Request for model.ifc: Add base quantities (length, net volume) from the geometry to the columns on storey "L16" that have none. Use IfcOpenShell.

First a look at what the model holds.

```python
import ifcopenshell
import ifcopenshell.util.element
import ifcopenshell.util.unit

model = ifcopenshell.open("model.ifc")
print(model.schema)
for unit_type in ("LENGTHUNIT", "AREAUNIT", "VOLUMEUNIT"):
    print(unit_type, ifcopenshell.util.unit.calculate_unit_scale(model, unit_type))
storey = next(s for s in model.by_type("IfcBuildingStorey") if s.Name == "L16")
columns = [e for e in ifcopenshell.util.element.get_decomposition(storey) if e.is_a("IfcColumn")]
for e in sorted(columns, key=lambda e: e.id()):
    print(e.id(), e.is_a(), e.Name, list(ifcopenshell.util.element.get_psets(e, qtos_only=True)), sep=" | ")
```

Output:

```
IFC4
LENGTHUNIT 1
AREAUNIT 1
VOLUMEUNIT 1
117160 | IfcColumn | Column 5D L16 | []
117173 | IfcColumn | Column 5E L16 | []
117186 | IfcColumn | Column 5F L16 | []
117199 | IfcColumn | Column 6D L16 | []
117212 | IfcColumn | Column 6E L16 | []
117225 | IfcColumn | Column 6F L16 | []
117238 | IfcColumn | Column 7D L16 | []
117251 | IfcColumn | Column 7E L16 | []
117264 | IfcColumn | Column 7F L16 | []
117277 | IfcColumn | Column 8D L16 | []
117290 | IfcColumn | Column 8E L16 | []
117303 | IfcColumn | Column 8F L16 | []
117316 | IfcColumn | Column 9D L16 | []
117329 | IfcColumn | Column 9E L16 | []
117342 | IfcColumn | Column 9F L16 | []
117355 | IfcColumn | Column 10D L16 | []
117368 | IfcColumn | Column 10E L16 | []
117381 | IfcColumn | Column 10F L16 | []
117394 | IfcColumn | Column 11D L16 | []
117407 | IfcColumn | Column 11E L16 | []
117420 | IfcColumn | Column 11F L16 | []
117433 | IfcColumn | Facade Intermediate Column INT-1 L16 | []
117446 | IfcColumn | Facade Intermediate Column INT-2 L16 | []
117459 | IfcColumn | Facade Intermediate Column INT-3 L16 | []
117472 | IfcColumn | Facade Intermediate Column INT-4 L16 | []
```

```python
import ifcopenshell
import ifcopenshell.api.pset
import ifcopenshell.geom
import ifcopenshell.util.element
import ifcopenshell.util.shape
import ifcopenshell.util.unit

model = ifcopenshell.open("model.ifc")
unit_scale = ifcopenshell.util.unit.calculate_unit_scale(model)
volume_scale = ifcopenshell.util.unit.calculate_unit_scale(model, "VOLUMEUNIT")
settings = ifcopenshell.geom.settings()

storey = next(s for s in model.by_type("IfcBuildingStorey") if s.Name == "L16")
columns = [e for e in ifcopenshell.util.element.get_decomposition(storey) if e.is_a("IfcColumn")]

for e in sorted(columns, key=lambda e: e.id()):
    if ifcopenshell.util.element.get_psets(e, qtos_only=True, should_inherit=False):
        continue
    # Geometry comes back in metres, in the element's own axes.
    shape = ifcopenshell.geom.create_shape(settings, e)
    values = {
        "Length": ifcopenshell.util.shape.get_z(shape.geometry) / unit_scale,
        "NetVolume": ifcopenshell.util.shape.get_volume(shape.geometry) / volume_scale,
    }
    qto = ifcopenshell.api.pset.add_qto(model, product=e, name="Qto_ColumnBaseQuantities")
    ifcopenshell.api.pset.edit_qto(model, qto=qto, properties=values)
    print(e.id(), {k: round(v, 3) for k, v in values.items()})

model.write("model-out.ifc")
```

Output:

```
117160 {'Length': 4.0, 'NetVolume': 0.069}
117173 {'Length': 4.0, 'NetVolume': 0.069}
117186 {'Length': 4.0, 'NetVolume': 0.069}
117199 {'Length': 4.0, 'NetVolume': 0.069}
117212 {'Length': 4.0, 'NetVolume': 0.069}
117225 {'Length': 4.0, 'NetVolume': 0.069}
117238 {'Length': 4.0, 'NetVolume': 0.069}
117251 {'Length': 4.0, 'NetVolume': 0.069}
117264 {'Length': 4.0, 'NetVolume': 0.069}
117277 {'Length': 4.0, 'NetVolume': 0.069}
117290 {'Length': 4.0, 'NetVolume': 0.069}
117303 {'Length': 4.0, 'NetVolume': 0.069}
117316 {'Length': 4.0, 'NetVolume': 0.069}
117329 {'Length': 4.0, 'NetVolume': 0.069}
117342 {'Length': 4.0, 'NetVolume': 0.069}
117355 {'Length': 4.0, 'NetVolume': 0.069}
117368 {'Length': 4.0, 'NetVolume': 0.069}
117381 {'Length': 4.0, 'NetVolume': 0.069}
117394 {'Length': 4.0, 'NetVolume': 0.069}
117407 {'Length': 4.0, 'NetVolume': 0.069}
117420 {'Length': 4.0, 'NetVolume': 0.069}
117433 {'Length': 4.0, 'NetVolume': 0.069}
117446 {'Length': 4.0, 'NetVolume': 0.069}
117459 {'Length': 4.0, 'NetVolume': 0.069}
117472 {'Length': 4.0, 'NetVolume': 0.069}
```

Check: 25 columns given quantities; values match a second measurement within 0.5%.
